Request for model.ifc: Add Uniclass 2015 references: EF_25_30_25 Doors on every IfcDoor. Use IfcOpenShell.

First a look at what the model holds.

```python
import ifcopenshell

model = ifcopenshell.open("model.ifc")
print(model.schema)
print("classifications:", [c.Name for c in model.by_type("IfcClassification")])
for ifc_class in ("IfcDoor", "IfcRoof", "IfcStair", "IfcWall", "IfcWindow"):
    print(ifc_class, len(model.by_type(ifc_class)))
```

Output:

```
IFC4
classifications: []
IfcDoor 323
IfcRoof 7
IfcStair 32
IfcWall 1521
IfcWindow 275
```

```python
import ifcopenshell
import ifcopenshell.api.classification

model = ifcopenshell.open("model.ifc")

system = ifcopenshell.api.classification.add_classification(model, classification="Uniclass 2015")

codes = {
    "IfcDoor": ("EF_25_30_25", "Doors"),
}
for ifc_class, (code, name) in codes.items():
    products = model.by_type(ifc_class)
    ifcopenshell.api.classification.add_reference(
        model, products=products, classification=system, identification=code, name=name
    )
    print(code, len(products))

model.write("model-out.ifc")
```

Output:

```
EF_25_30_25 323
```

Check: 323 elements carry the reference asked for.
